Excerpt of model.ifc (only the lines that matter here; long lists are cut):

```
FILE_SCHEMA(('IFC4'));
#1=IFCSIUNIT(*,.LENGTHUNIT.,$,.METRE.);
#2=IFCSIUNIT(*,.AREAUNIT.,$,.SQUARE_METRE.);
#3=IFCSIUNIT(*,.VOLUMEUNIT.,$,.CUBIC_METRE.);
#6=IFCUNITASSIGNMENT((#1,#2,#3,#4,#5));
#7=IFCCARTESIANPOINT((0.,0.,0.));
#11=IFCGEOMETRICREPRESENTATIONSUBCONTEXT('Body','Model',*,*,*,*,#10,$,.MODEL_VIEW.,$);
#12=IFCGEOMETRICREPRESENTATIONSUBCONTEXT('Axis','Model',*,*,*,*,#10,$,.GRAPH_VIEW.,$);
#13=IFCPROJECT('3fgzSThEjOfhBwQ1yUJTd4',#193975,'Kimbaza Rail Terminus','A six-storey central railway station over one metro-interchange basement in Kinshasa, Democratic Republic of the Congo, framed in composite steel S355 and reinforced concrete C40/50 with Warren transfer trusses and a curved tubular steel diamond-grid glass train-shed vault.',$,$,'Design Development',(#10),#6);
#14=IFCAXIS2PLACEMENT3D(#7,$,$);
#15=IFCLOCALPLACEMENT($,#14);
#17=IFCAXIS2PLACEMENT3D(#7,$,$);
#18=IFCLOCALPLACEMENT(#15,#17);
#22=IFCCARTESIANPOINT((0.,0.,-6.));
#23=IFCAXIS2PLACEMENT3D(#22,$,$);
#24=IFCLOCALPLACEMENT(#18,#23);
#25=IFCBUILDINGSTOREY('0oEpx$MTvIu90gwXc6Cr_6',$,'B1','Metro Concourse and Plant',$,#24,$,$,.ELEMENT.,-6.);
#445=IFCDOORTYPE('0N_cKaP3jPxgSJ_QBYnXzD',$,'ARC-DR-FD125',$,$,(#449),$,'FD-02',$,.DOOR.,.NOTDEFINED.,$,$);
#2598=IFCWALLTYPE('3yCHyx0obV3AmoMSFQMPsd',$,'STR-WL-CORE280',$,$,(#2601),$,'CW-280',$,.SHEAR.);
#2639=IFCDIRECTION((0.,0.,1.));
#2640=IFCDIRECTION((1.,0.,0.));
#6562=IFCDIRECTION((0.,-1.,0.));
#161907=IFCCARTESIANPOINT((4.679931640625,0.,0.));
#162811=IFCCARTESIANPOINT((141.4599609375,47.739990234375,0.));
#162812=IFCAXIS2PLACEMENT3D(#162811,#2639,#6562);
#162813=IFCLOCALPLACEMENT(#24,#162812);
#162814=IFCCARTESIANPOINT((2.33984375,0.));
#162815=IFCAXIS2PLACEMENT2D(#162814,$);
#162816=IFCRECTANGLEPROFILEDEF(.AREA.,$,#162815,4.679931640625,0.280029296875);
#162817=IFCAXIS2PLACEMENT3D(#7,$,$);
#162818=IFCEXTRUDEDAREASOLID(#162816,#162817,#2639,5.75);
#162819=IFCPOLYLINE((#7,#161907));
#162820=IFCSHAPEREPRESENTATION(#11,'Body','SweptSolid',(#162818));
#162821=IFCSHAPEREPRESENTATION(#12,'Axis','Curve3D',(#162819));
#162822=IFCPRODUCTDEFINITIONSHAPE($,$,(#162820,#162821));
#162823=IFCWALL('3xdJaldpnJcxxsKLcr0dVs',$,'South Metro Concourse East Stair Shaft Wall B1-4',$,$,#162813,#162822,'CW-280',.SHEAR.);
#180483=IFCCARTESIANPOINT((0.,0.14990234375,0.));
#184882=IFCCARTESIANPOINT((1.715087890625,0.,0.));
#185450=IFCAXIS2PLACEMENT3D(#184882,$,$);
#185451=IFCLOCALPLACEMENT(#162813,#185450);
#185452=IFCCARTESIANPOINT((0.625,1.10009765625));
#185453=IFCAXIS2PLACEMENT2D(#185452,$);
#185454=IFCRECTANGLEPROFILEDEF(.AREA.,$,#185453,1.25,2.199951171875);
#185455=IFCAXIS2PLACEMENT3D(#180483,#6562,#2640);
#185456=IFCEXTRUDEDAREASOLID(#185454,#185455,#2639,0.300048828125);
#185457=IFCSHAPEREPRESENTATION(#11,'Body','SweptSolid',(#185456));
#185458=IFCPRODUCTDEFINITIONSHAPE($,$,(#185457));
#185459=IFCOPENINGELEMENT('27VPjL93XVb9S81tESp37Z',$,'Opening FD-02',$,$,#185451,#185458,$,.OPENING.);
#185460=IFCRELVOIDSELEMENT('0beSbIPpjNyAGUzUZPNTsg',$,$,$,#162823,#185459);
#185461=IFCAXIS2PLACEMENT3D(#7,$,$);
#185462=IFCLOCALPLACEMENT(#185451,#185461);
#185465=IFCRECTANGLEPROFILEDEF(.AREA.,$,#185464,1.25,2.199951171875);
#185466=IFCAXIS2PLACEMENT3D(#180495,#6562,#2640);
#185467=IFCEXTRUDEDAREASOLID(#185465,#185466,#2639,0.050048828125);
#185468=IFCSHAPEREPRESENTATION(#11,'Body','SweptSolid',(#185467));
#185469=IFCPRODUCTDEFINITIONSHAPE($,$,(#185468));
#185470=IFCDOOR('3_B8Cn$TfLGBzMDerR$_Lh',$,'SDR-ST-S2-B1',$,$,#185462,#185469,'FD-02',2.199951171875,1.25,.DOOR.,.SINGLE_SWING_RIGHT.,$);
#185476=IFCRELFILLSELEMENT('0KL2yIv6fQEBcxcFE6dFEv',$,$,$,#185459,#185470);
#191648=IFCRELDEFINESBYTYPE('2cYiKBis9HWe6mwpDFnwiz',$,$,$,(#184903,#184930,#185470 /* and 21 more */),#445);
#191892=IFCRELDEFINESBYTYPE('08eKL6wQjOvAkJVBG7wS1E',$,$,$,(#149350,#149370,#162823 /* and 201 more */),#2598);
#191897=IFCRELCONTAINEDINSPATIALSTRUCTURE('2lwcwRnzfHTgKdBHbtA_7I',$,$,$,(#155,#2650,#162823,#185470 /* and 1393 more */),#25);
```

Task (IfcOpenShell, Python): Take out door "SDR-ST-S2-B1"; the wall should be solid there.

```python
import ifcopenshell
import ifcopenshell.api.feature
import ifcopenshell.api.root
import ifcopenshell.geom
import ifcopenshell.util.shape

model = ifcopenshell.open("model.ifc")
settings = ifcopenshell.geom.settings()


def volume(element):
    """Net volume in cubic metres, openings subtracted."""
    shape = ifcopenshell.geom.create_shape(settings, element)
    return ifcopenshell.util.shape.get_volume(shape.geometry)


door = model.by_id(185470)
opening = door.FillsVoids[0].RelatingOpeningElement
wall = opening.VoidsElements[0].RelatingBuildingElement
before = volume(wall)

ifcopenshell.api.root.remove_product(model, product=door)
ifcopenshell.api.feature.remove_feature(model, feature=opening)

after = volume(wall)

print(f"wall volume {before:.3f} -> {after:.3f} m3")

model.write("model_edited.ifc")
```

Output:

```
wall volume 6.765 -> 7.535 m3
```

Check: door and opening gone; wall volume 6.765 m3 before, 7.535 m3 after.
